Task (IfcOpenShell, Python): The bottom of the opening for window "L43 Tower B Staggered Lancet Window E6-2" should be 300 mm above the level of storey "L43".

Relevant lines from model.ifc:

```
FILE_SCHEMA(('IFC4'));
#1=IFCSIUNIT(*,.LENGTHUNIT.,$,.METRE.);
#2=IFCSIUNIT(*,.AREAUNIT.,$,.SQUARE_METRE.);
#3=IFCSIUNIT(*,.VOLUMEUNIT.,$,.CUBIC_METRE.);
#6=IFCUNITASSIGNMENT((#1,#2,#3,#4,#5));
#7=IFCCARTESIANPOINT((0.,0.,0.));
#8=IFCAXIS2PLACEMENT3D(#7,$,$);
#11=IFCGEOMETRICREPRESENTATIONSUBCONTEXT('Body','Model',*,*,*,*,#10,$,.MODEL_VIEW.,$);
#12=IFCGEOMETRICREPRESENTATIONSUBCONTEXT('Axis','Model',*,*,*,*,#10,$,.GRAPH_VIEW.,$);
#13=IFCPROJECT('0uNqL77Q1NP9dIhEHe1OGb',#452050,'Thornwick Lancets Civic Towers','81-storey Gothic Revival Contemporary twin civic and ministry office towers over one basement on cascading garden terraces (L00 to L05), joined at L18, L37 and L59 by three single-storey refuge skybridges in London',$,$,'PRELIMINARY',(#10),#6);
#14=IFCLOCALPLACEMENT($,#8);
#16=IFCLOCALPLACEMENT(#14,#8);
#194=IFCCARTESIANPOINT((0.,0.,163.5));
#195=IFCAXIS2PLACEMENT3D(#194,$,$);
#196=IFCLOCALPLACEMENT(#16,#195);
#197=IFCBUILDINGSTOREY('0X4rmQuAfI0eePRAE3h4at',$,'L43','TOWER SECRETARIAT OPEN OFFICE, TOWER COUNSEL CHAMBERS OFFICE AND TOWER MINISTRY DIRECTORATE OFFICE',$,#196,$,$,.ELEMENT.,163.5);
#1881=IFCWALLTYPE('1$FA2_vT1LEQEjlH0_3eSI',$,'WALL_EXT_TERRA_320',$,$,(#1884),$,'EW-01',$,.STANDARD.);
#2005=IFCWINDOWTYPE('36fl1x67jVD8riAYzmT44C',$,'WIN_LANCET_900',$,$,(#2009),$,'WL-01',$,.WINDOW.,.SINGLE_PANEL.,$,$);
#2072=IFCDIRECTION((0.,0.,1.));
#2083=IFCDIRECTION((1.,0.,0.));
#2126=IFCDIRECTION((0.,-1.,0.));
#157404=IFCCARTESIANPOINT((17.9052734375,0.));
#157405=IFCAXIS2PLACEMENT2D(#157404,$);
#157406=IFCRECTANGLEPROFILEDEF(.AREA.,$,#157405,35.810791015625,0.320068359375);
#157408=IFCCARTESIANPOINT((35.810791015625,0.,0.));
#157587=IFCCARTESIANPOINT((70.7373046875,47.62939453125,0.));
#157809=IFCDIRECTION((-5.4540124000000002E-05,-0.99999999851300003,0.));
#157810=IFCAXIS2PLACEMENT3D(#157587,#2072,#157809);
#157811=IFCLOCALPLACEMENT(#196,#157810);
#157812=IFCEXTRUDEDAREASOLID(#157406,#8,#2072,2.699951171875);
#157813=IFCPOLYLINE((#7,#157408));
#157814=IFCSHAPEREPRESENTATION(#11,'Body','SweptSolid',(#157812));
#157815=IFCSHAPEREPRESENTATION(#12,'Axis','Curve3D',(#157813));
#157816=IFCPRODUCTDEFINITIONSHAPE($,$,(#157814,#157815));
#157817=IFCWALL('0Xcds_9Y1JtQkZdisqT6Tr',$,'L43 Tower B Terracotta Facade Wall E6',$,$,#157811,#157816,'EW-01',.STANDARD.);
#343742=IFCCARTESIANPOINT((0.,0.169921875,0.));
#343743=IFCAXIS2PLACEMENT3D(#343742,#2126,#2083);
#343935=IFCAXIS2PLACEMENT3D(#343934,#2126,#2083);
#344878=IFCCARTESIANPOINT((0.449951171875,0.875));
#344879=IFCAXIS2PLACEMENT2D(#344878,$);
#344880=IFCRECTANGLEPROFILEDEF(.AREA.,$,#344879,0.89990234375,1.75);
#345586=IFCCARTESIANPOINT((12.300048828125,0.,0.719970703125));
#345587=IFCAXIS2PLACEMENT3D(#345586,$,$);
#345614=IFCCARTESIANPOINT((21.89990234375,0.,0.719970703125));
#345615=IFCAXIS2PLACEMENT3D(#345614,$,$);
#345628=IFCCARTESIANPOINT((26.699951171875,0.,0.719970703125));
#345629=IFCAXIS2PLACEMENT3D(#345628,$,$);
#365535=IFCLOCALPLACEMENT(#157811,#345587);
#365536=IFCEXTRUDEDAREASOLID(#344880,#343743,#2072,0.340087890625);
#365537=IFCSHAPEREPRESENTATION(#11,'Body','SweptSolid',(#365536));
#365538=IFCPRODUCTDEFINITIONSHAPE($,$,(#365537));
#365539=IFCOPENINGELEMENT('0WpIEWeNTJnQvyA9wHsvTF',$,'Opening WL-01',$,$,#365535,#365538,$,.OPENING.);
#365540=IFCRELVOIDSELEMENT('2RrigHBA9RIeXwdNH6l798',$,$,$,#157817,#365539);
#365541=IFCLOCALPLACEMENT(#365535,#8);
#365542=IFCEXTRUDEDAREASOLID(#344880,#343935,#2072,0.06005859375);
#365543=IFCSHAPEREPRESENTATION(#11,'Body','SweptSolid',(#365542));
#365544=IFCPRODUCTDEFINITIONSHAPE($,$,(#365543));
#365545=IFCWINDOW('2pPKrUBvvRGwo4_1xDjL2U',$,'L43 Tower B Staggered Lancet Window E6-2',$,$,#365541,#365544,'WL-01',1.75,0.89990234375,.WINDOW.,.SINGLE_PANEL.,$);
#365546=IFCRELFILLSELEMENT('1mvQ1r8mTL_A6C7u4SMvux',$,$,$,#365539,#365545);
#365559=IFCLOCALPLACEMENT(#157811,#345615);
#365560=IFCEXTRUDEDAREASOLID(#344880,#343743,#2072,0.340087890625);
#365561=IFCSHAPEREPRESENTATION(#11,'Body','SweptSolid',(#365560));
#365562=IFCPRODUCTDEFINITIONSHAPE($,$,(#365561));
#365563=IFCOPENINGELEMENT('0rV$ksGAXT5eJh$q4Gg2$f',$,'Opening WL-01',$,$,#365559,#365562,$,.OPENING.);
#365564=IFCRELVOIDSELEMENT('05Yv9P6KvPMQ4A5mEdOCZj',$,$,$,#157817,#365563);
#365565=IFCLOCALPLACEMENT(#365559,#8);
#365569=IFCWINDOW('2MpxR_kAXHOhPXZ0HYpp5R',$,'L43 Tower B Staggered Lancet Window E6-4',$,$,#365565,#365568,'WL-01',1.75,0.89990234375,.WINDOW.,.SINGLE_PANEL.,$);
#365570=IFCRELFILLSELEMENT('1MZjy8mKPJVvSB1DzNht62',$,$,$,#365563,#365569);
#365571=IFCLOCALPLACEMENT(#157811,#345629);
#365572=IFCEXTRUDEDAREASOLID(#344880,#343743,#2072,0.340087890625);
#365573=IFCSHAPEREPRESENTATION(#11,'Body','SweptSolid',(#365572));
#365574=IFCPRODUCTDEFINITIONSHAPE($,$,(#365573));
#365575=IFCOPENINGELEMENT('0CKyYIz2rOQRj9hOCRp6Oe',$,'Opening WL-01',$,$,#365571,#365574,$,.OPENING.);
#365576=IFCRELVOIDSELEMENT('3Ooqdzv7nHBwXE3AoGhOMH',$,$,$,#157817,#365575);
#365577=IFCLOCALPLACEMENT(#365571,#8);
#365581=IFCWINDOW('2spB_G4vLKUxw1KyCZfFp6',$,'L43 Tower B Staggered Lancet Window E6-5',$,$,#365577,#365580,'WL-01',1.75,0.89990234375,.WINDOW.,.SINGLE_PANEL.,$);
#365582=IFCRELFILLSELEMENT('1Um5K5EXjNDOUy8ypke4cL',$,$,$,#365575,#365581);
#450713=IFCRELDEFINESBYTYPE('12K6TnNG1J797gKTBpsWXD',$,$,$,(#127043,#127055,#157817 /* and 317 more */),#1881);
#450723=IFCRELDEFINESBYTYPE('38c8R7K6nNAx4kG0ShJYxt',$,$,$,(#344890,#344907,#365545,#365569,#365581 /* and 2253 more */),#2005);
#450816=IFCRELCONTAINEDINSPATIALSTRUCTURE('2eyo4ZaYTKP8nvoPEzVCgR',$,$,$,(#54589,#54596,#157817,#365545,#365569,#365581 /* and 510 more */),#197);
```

```python
import numpy as np
import ifcopenshell
import ifcopenshell.api.geometry
import ifcopenshell.geom
import ifcopenshell.util.element
import ifcopenshell.util.placement
import ifcopenshell.util.shape
import ifcopenshell.util.unit

model = ifcopenshell.open("model.ifc")
unit_scale = ifcopenshell.util.unit.calculate_unit_scale(model)

window = model.by_guid("2pPKrUBvvRGwo4_1xDjL2U")
opening = window.FillsVoids[0].RelatingOpeningElement
storey = ifcopenshell.util.element.get_container(window, ifc_class="IfcBuildingStorey")
level = ifcopenshell.util.placement.get_local_placement(storey.ObjectPlacement)[2, 3]

# The opening's origin need not be at the sill, so measure its lowest point.
shape = ifcopenshell.geom.create_shape(ifcopenshell.geom.settings(), opening)
bottom = ifcopenshell.util.shape.get_shape_bottom_elevation(shape, shape.geometry) / unit_scale
dz = level + 0.3 / unit_scale - bottom

shift = np.array([0.0, 0.0, dz])
# The window is placed relative to its opening, so it follows when the opening moves.
matrix = ifcopenshell.util.placement.get_local_placement(opening.ObjectPlacement)
matrix[:3, 3] += shift
ifcopenshell.api.geometry.edit_object_placement(
    model, product=opening, matrix=matrix, is_si=False, should_transform_children=True
)

print(f"moved by {dz * unit_scale:+.3f} m")

model.write("model-out.ifc")
```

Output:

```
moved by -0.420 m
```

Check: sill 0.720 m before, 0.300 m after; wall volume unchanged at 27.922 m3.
